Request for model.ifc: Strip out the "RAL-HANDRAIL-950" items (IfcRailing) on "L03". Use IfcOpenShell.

First a look at what the model holds.

```python
import ifcopenshell
import ifcopenshell.util.element

model = ifcopenshell.open("model.ifc")
print(model.schema)
storey = next(s for s in model.by_type("IfcBuildingStorey") if s.Name == "L03")
railings = [e for e in ifcopenshell.util.element.get_decomposition(storey) if e.is_a("IfcRailing")]
seen = {}
for e in railings:
    element_type = ifcopenshell.util.element.get_type(e)
    name = element_type.Name if element_type not in (None, e) else None
    seen[name] = seen.get(name, 0) + 1
for name, count in sorted(seen.items(), key=str):
    print(count, "x", name)
```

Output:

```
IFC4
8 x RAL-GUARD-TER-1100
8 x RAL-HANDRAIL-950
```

```python
import ifcopenshell
import ifcopenshell.api.root
import ifcopenshell.util.element

model = ifcopenshell.open("model.ifc")

storey = next(s for s in model.by_type("IfcBuildingStorey") if s.Name == "L03")
railings = [e for e in ifcopenshell.util.element.get_decomposition(storey) if e.is_a("IfcRailing")]
targets = [e for e in railings if (t := ifcopenshell.util.element.get_type(e)) not in (None, e) and t.Name == "RAL-HANDRAIL-950"]

for e in targets:
    ifcopenshell.api.root.remove_product(model, product=e)
print(len(targets), "removed")

model.write("model_rev.ifc")
```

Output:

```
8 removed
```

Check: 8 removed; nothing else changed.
